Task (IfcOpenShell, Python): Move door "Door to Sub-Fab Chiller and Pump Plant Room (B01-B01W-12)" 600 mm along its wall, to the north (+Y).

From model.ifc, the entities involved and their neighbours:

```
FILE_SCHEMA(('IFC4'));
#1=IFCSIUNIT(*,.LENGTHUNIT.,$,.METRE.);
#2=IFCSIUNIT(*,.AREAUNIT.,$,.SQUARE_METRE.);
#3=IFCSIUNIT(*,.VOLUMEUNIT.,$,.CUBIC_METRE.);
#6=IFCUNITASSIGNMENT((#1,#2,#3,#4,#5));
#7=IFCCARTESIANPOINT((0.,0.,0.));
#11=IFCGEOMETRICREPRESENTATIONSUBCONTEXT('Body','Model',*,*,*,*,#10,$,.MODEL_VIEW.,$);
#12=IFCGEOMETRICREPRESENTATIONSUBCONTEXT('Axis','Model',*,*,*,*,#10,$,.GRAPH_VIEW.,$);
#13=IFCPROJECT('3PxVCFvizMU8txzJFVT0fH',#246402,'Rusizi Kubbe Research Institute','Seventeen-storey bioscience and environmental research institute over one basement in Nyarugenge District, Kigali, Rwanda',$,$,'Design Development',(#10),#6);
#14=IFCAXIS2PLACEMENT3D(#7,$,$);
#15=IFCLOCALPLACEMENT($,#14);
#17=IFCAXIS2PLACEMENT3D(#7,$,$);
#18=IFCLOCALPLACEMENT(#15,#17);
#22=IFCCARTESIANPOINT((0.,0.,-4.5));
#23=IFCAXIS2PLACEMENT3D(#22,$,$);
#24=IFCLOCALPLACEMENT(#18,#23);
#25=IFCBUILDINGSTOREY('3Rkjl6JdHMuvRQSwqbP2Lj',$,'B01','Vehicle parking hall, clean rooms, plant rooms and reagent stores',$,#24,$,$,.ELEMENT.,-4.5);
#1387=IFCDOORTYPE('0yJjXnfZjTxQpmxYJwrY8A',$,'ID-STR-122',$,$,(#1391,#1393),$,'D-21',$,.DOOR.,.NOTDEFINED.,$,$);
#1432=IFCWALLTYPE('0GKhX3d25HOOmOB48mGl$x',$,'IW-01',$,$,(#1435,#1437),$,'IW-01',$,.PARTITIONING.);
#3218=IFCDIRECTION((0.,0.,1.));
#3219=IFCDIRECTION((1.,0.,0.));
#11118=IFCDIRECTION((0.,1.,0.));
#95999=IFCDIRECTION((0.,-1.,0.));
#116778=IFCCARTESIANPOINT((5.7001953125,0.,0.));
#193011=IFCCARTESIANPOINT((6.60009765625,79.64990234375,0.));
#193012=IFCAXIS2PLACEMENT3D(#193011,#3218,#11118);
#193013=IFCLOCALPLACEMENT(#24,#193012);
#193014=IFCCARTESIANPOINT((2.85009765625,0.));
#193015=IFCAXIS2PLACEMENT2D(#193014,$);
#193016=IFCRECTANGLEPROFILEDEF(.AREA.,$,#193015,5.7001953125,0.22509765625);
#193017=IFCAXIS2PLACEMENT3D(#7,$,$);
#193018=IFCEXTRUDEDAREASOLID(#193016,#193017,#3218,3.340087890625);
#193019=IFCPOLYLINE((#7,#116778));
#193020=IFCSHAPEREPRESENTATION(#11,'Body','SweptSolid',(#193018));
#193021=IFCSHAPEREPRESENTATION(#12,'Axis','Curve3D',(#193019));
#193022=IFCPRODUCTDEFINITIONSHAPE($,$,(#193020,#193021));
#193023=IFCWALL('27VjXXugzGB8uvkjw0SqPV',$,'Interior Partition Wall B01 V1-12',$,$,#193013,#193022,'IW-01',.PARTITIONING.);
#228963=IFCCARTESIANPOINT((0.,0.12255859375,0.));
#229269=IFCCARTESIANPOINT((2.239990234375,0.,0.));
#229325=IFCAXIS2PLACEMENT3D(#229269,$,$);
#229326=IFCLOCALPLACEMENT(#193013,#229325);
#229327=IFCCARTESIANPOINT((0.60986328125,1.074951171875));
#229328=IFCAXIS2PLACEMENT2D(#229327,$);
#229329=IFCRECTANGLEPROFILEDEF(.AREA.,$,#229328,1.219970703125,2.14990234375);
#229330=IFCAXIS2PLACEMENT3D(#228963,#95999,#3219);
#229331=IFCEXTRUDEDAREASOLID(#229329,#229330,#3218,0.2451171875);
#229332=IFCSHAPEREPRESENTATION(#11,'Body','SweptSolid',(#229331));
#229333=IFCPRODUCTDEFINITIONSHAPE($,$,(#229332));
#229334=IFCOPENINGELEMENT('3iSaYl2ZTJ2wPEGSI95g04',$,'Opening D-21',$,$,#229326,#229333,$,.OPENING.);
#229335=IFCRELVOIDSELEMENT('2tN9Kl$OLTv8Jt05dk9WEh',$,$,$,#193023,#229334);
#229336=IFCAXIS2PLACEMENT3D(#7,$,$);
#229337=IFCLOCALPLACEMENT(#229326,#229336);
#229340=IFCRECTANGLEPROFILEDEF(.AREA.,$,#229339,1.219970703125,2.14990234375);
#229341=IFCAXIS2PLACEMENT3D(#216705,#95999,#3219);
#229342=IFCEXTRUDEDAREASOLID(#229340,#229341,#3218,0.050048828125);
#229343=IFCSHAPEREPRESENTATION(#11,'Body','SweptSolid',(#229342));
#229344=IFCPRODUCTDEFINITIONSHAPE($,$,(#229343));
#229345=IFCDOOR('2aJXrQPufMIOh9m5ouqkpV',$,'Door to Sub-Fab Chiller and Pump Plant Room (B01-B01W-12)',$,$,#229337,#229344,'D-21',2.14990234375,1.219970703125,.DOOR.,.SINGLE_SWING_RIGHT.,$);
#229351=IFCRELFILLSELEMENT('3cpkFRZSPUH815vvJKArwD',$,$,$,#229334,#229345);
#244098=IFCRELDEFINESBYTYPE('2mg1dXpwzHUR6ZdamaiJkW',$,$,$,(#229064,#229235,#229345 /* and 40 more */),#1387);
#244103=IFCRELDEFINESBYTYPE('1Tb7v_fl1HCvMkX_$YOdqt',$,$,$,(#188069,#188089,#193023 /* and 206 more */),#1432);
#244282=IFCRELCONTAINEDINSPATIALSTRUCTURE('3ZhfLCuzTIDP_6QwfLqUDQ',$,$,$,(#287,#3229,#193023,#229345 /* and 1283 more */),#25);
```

```python
import ifcopenshell
import ifcopenshell.api.geometry
import ifcopenshell.util.placement

model = ifcopenshell.open("model.ifc")

door = model.by_id(229345)
opening = door.FillsVoids[0].RelatingOpeningElement
wall = opening.VoidsElements[0].RelatingBuildingElement

wall_matrix = ifcopenshell.util.placement.get_local_placement(wall.ObjectPlacement)
shift = wall_matrix[:3, 0] * 0.6
before = ifcopenshell.util.placement.get_local_placement(door.ObjectPlacement)[:3, 3].copy()

# The door is placed relative to its opening, so it follows when the opening moves.
matrix = ifcopenshell.util.placement.get_local_placement(opening.ObjectPlacement)
matrix[:3, 3] += shift
ifcopenshell.api.geometry.edit_object_placement(
    model, product=opening, matrix=matrix, is_si=False, should_transform_children=True
)

after = ifcopenshell.util.placement.get_local_placement(door.ObjectPlacement)[:3, 3]
print("door moved by", (after - before).round(3) + 0.0)

model.write("model_edited.ifc")
```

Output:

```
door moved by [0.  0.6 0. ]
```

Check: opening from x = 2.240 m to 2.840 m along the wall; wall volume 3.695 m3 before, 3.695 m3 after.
